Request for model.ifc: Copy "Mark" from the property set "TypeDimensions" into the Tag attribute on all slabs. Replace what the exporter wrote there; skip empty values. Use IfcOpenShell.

First a look at what the model holds.

```python
import ifcopenshell
import ifcopenshell.util.element

model = ifcopenshell.open("model.ifc")
print(model.schema)
slabs = model.by_type("IfcSlab")
print(len(slabs), "slabs")
for e in slabs[:8]:
    source = ifcopenshell.util.element.get_pset(e, "TypeDimensions", "Mark")
    target = e.Tag
    print(e.id(), repr(source), repr(target), sep=" | ")
```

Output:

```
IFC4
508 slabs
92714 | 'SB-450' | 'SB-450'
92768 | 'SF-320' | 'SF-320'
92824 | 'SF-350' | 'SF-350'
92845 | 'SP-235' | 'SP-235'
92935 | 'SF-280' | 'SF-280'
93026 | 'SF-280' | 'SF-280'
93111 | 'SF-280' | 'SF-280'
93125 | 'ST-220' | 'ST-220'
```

```python
import ifcopenshell
import ifcopenshell.util.element

model = ifcopenshell.open("model.ifc")

count = 0
for e in model.by_type("IfcSlab"):
    value = ifcopenshell.util.element.get_pset(e, "TypeDimensions", "Mark")
    current = e.Tag
    if not value or not value.strip() or current == value:
        continue
    e.Tag = value
    count += 1

print(count, "slabs updated")

model.write("model_v2.ifc")
```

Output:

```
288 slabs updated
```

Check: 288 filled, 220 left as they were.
